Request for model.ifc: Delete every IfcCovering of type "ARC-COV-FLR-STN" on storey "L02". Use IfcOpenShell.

First a look at what the model holds.

```python
import ifcopenshell
import ifcopenshell.util.element

model = ifcopenshell.open("model.ifc")
print(model.schema)
storey = next(s for s in model.by_type("IfcBuildingStorey") if s.Name == "L02")
coverings = [e for e in ifcopenshell.util.element.get_decomposition(storey) if e.is_a("IfcCovering")]
seen = {}
for e in coverings:
    element_type = ifcopenshell.util.element.get_type(e)
    name = element_type.Name if element_type not in (None, e) else None
    seen[name] = seen.get(name, 0) + 1
for name, count in sorted(seen.items(), key=str):
    print(count, "x", name)
```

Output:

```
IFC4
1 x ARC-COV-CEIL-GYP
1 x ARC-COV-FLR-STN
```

```python
import ifcopenshell
import ifcopenshell.api.root
import ifcopenshell.util.element

model = ifcopenshell.open("model.ifc")

storey = next(s for s in model.by_type("IfcBuildingStorey") if s.Name == "L02")
coverings = [e for e in ifcopenshell.util.element.get_decomposition(storey) if e.is_a("IfcCovering")]
targets = [e for e in coverings if (t := ifcopenshell.util.element.get_type(e)) not in (None, e) and t.Name == "ARC-COV-FLR-STN"]

for e in targets:
    ifcopenshell.api.root.remove_product(model, product=e)
print(len(targets), "removed")

model.write("model_rev.ifc")
```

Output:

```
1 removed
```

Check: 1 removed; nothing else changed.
